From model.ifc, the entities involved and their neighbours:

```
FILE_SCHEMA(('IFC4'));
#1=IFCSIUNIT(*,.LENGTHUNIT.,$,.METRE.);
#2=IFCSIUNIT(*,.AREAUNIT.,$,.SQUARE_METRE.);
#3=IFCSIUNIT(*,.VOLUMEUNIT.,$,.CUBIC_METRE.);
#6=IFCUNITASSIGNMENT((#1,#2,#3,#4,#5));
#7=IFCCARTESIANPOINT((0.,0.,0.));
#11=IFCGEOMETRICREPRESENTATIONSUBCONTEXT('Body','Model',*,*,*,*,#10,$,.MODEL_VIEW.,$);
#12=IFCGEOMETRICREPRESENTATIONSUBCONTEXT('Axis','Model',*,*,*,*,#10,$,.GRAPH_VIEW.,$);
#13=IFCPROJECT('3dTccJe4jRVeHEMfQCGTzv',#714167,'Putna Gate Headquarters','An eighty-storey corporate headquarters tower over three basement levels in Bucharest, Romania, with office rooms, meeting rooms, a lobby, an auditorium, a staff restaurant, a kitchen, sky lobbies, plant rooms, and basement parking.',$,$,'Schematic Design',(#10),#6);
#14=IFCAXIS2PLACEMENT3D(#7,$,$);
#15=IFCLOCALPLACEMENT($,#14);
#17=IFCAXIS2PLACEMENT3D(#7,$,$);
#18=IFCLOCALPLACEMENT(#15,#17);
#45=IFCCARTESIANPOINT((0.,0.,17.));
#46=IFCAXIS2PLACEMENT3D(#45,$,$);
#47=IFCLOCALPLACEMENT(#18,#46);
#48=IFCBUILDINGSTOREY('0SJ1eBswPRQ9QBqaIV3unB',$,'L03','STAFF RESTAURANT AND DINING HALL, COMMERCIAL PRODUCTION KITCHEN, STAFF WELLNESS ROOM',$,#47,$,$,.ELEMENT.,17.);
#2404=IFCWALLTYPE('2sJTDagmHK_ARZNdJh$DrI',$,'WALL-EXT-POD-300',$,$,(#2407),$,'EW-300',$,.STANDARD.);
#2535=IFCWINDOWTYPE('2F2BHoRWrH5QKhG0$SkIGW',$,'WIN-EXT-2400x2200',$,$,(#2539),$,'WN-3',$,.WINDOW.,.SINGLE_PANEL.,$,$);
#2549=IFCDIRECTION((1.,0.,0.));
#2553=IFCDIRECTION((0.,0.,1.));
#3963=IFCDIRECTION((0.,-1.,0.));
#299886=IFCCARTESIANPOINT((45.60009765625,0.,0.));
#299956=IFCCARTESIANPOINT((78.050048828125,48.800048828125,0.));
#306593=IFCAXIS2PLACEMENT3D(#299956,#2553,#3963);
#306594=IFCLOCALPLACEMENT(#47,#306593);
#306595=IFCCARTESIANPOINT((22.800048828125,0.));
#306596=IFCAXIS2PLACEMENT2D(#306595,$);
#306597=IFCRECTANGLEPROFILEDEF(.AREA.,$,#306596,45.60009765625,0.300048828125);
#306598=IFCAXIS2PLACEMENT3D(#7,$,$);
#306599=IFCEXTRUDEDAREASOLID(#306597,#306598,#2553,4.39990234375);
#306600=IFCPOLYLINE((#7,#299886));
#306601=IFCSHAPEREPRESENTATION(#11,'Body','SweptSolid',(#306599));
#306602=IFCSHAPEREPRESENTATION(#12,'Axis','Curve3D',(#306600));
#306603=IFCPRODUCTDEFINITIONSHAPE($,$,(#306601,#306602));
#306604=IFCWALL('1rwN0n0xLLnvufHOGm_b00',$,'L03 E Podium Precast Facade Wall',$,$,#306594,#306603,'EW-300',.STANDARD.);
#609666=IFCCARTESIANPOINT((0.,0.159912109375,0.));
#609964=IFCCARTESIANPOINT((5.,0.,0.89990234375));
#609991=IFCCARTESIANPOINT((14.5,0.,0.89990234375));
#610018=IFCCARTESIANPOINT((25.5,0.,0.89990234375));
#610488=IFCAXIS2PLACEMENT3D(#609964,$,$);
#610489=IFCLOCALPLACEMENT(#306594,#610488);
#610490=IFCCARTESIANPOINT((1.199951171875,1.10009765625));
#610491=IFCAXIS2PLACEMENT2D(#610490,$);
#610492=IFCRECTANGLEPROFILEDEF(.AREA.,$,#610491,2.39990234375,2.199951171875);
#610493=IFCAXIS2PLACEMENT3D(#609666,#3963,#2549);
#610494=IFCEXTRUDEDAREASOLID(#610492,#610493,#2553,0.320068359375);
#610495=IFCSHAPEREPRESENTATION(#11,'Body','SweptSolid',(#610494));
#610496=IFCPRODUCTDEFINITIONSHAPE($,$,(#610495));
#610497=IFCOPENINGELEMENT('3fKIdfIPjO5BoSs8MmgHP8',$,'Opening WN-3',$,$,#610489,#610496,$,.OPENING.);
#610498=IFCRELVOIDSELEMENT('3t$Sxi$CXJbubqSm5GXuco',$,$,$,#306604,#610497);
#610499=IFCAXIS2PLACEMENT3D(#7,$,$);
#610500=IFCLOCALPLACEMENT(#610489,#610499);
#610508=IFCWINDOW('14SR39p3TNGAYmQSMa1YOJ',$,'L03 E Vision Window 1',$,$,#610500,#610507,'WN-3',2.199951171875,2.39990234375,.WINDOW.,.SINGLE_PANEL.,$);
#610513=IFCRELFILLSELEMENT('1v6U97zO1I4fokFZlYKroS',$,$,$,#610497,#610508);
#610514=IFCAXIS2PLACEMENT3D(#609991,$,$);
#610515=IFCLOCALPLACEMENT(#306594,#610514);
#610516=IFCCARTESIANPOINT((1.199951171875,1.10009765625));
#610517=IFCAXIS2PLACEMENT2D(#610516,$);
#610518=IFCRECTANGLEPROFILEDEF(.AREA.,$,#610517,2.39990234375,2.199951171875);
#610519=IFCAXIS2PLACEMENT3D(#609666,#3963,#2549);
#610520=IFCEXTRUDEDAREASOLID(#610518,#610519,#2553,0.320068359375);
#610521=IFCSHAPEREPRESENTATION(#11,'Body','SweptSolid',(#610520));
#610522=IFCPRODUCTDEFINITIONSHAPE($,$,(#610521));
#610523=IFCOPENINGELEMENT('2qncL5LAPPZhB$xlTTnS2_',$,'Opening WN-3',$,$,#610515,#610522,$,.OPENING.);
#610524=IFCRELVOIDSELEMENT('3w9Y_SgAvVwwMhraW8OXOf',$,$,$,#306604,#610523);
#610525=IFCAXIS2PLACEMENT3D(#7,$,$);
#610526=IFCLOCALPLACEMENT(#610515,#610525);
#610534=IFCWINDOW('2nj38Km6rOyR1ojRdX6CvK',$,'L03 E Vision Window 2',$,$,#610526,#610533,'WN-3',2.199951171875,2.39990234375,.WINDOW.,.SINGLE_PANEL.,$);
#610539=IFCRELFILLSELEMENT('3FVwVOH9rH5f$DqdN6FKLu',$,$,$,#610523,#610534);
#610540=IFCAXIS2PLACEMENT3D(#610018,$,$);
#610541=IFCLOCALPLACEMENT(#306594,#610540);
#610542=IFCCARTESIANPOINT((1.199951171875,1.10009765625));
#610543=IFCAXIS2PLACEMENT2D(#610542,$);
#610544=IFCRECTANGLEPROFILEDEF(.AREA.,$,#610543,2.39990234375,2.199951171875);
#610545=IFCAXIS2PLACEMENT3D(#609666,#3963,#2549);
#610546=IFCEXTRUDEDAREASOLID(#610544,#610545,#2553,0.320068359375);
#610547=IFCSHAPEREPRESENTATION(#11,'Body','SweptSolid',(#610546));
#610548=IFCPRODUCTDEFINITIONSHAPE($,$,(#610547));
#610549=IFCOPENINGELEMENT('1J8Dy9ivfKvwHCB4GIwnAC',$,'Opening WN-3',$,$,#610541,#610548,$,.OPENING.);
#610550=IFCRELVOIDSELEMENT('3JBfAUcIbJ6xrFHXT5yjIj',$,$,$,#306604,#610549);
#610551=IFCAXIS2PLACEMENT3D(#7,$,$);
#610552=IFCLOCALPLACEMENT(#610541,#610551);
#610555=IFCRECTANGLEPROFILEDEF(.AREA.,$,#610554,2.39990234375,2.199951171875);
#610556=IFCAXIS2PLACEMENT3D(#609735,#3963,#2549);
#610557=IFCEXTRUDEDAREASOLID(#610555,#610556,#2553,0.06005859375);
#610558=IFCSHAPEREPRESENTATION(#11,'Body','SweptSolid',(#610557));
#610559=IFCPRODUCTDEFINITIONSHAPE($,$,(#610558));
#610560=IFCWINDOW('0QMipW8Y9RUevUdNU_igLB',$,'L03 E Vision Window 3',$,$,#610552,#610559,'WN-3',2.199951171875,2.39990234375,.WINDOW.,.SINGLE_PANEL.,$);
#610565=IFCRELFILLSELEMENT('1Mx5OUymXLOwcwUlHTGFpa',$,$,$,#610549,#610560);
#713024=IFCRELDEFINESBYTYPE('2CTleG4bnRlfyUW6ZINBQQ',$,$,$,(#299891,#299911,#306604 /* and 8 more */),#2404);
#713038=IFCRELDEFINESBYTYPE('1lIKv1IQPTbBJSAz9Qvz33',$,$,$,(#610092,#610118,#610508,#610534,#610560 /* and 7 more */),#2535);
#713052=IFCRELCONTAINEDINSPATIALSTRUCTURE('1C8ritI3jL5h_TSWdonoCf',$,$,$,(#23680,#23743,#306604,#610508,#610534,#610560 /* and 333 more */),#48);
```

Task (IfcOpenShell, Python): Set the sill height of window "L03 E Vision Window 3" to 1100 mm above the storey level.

```python
import numpy as np
import ifcopenshell
import ifcopenshell.api.geometry
import ifcopenshell.geom
import ifcopenshell.util.element
import ifcopenshell.util.placement
import ifcopenshell.util.shape
import ifcopenshell.util.unit

model = ifcopenshell.open("model.ifc")
unit_scale = ifcopenshell.util.unit.calculate_unit_scale(model)

window = model.by_guid("0QMipW8Y9RUevUdNU_igLB")
opening = window.FillsVoids[0].RelatingOpeningElement
storey = ifcopenshell.util.element.get_container(window, ifc_class="IfcBuildingStorey")
level = ifcopenshell.util.placement.get_local_placement(storey.ObjectPlacement)[2, 3]

# The opening's origin need not be at the sill, so measure its lowest point.
shape = ifcopenshell.geom.create_shape(ifcopenshell.geom.settings(), opening)
bottom = ifcopenshell.util.shape.get_shape_bottom_elevation(shape, shape.geometry) / unit_scale
dz = level + 1.1 / unit_scale - bottom

shift = np.array([0.0, 0.0, dz])
# The window is placed relative to its opening, so it follows when the opening moves.
matrix = ifcopenshell.util.placement.get_local_placement(opening.ObjectPlacement)
matrix[:3, 3] += shift
ifcopenshell.api.geometry.edit_object_placement(
    model, product=opening, matrix=matrix, is_si=False, should_transform_children=True
)

print(f"moved by {dz * unit_scale:+.3f} m")

model.write("model_updated.ifc")
```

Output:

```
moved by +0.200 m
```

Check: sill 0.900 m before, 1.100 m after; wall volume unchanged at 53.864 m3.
